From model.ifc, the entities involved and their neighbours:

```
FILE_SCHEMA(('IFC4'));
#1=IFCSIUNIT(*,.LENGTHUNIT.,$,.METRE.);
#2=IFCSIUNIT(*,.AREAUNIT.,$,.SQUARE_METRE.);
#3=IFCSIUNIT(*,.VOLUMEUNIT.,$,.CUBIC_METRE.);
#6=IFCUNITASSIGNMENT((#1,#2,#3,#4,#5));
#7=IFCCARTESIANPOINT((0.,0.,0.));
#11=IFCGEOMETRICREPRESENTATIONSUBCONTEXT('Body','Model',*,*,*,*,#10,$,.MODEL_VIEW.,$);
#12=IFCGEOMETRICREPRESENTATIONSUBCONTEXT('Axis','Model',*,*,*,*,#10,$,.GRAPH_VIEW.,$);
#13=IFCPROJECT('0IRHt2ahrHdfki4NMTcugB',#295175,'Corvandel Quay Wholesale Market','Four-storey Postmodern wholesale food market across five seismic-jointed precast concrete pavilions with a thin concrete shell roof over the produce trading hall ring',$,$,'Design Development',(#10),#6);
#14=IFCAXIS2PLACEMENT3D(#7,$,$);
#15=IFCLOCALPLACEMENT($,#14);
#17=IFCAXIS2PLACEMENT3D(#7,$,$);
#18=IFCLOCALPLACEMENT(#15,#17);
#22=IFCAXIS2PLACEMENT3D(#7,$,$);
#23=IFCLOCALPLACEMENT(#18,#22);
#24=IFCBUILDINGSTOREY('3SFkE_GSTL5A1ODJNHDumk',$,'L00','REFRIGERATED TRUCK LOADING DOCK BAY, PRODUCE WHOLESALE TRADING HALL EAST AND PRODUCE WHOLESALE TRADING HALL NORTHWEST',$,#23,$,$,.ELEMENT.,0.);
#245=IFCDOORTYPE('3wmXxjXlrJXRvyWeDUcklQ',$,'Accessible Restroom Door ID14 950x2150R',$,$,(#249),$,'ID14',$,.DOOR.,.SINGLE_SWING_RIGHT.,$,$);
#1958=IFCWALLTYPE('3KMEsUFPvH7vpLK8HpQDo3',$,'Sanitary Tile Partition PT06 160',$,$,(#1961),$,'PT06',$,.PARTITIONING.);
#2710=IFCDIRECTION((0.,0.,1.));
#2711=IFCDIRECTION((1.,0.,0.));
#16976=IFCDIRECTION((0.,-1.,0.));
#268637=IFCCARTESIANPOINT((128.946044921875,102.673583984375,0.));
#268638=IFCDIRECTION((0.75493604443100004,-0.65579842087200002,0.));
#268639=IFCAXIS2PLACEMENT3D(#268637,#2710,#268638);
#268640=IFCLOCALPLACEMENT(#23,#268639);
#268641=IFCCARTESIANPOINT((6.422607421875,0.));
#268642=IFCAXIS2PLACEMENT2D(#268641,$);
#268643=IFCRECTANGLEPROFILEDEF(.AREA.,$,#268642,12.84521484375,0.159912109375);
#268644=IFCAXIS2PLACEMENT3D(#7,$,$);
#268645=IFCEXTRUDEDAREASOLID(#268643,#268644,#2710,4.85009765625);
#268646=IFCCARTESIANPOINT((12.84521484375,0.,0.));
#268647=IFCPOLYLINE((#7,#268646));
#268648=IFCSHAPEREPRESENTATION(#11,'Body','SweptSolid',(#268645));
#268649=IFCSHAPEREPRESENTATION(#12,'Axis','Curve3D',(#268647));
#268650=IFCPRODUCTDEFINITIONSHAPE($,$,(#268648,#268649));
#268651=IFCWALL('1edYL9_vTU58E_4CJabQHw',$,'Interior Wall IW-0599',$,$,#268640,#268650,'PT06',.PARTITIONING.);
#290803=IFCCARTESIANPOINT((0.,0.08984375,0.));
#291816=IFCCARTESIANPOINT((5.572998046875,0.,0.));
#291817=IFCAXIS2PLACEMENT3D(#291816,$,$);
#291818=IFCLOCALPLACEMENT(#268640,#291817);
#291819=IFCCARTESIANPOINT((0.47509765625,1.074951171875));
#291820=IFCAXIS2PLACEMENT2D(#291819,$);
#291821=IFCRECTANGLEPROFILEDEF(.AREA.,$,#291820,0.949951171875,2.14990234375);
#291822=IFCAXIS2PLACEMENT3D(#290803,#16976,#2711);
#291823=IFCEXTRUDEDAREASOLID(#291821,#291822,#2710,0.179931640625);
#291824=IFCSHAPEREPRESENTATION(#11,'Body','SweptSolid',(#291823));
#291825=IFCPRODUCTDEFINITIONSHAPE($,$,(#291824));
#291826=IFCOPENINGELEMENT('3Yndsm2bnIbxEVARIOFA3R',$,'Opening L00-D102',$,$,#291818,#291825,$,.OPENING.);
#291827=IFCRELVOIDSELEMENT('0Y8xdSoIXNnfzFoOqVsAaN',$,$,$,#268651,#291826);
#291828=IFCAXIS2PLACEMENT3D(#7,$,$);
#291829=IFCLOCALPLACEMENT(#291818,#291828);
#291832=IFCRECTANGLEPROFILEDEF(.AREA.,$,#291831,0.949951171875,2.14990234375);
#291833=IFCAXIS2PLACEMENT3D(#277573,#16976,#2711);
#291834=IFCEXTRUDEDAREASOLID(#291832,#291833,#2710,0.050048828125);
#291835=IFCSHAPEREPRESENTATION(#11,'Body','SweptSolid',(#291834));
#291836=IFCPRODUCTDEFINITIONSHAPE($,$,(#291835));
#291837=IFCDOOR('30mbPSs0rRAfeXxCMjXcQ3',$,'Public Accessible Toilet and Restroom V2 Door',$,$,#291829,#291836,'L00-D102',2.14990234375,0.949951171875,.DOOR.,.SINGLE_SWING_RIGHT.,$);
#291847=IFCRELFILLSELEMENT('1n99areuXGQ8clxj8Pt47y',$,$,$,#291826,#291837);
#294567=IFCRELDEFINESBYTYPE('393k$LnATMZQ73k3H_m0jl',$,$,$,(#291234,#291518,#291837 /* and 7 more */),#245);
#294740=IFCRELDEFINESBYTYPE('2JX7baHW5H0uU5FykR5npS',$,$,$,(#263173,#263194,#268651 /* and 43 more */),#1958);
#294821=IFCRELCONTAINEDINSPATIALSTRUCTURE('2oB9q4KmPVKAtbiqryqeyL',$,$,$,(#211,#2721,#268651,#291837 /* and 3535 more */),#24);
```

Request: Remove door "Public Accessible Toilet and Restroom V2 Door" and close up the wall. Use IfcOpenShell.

```python
import ifcopenshell
import ifcopenshell.api.feature
import ifcopenshell.api.root
import ifcopenshell.geom
import ifcopenshell.util.shape

model = ifcopenshell.open("model.ifc")
settings = ifcopenshell.geom.settings()


def volume(element):
    """Net volume in cubic metres, openings subtracted."""
    shape = ifcopenshell.geom.create_shape(settings, element)
    return ifcopenshell.util.shape.get_volume(shape.geometry)


door = model.by_id(291837)
opening = door.FillsVoids[0].RelatingOpeningElement
wall = opening.VoidsElements[0].RelatingBuildingElement
before = volume(wall)

ifcopenshell.api.root.remove_product(model, product=door)
ifcopenshell.api.feature.remove_feature(model, feature=opening)

after = volume(wall)

print(f"wall volume {before:.3f} -> {after:.3f} m3")

model.write("model_edited.ifc")
```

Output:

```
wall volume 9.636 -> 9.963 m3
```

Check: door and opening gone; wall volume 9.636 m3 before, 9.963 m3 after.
